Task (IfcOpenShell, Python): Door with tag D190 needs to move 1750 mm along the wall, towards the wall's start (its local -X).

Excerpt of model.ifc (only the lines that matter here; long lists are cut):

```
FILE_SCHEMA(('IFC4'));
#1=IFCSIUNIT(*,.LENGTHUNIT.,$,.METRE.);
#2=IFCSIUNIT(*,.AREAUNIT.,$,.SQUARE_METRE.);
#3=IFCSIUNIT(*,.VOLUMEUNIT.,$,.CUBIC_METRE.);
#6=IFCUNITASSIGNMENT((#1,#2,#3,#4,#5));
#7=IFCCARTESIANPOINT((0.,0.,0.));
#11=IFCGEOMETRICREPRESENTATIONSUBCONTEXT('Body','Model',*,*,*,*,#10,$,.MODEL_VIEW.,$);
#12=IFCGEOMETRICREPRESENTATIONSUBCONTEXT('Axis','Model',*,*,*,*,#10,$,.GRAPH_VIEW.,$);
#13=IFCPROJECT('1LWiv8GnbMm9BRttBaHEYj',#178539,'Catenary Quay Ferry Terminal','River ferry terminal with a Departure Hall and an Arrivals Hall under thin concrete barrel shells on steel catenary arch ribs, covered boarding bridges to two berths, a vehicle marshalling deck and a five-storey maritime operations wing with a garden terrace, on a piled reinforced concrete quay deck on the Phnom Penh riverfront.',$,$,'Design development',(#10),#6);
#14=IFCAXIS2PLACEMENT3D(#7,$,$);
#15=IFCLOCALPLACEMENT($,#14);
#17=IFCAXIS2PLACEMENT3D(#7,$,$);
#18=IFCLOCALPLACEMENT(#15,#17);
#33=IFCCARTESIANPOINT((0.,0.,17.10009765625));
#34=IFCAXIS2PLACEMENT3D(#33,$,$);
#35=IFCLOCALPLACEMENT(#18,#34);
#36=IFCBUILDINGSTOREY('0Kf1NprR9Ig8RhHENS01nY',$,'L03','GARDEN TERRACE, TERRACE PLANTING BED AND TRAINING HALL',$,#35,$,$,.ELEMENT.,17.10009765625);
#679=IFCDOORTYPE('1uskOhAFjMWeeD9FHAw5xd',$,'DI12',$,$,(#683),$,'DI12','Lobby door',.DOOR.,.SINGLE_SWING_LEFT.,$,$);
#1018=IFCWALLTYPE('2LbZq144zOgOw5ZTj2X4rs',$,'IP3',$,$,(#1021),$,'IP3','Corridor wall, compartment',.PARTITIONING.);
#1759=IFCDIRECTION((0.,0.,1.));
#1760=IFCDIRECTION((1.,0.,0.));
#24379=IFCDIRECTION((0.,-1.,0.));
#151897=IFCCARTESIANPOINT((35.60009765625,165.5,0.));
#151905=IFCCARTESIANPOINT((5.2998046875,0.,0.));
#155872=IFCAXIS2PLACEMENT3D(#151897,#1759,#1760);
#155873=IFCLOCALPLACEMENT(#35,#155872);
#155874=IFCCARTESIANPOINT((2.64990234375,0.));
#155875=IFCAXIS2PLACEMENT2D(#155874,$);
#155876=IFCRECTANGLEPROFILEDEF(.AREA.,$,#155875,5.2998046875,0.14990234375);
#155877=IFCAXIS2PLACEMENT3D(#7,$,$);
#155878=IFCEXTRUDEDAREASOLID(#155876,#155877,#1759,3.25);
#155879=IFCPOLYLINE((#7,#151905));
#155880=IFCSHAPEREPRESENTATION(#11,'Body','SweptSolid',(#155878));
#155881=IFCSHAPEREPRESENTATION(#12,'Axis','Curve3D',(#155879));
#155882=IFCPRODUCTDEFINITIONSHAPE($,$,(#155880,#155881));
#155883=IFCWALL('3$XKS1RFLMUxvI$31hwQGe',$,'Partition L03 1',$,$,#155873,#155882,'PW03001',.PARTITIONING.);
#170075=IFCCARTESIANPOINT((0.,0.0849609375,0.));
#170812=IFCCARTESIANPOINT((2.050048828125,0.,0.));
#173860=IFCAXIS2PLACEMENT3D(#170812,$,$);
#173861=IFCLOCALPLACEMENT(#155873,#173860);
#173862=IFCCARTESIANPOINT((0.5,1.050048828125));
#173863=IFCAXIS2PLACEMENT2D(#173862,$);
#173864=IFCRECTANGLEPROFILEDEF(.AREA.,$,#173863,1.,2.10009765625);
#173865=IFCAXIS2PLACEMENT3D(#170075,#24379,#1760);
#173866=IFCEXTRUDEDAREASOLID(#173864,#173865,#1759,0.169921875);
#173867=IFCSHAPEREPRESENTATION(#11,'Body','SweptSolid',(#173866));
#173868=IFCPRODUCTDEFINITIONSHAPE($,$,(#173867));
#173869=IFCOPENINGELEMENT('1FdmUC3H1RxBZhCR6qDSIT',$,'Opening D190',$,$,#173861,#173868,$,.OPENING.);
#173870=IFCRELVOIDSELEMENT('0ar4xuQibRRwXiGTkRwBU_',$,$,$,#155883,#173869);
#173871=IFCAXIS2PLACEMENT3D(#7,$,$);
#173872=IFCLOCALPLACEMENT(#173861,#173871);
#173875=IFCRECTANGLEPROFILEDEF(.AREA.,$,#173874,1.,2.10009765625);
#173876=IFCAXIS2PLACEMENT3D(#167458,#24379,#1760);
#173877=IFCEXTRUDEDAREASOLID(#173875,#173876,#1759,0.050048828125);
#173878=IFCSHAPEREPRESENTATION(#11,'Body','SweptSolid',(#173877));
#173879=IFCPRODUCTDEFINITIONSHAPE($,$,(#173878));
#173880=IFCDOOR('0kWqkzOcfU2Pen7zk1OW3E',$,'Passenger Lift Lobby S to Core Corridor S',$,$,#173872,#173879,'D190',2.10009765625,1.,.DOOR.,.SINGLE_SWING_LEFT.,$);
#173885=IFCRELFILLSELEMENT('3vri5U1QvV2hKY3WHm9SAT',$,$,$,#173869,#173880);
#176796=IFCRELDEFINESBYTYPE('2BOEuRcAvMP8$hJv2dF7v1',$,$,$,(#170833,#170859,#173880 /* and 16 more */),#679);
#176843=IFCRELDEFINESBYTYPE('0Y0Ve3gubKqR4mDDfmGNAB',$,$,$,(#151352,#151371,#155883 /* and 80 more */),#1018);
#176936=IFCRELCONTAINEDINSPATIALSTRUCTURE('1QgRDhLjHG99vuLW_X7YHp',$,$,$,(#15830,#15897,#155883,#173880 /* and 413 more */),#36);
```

```python
import ifcopenshell
import ifcopenshell.api.geometry
import ifcopenshell.util.placement
import ifcopenshell.util.unit

model = ifcopenshell.open("model.ifc")
unit_scale = ifcopenshell.util.unit.calculate_unit_scale(model)

door = model.by_guid("0kWqkzOcfU2Pen7zk1OW3E")
opening = door.FillsVoids[0].RelatingOpeningElement
wall = opening.VoidsElements[0].RelatingBuildingElement

wall_matrix = ifcopenshell.util.placement.get_local_placement(wall.ObjectPlacement)
shift = wall_matrix[:3, 0] * -1.75 / unit_scale
before = ifcopenshell.util.placement.get_local_placement(door.ObjectPlacement)[:3, 3].copy()

# The door is placed relative to its opening, so it follows when the opening moves.
matrix = ifcopenshell.util.placement.get_local_placement(opening.ObjectPlacement)
matrix[:3, 3] += shift
ifcopenshell.api.geometry.edit_object_placement(
    model, product=opening, matrix=matrix, is_si=False, should_transform_children=True
)

after = ifcopenshell.util.placement.get_local_placement(door.ObjectPlacement)[:3, 3]
print("door moved by", (after - before).round(3) + 0.0)

model.write("model_rev.ifc")
```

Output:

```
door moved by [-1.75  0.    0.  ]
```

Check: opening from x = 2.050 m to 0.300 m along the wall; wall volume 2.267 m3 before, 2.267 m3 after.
